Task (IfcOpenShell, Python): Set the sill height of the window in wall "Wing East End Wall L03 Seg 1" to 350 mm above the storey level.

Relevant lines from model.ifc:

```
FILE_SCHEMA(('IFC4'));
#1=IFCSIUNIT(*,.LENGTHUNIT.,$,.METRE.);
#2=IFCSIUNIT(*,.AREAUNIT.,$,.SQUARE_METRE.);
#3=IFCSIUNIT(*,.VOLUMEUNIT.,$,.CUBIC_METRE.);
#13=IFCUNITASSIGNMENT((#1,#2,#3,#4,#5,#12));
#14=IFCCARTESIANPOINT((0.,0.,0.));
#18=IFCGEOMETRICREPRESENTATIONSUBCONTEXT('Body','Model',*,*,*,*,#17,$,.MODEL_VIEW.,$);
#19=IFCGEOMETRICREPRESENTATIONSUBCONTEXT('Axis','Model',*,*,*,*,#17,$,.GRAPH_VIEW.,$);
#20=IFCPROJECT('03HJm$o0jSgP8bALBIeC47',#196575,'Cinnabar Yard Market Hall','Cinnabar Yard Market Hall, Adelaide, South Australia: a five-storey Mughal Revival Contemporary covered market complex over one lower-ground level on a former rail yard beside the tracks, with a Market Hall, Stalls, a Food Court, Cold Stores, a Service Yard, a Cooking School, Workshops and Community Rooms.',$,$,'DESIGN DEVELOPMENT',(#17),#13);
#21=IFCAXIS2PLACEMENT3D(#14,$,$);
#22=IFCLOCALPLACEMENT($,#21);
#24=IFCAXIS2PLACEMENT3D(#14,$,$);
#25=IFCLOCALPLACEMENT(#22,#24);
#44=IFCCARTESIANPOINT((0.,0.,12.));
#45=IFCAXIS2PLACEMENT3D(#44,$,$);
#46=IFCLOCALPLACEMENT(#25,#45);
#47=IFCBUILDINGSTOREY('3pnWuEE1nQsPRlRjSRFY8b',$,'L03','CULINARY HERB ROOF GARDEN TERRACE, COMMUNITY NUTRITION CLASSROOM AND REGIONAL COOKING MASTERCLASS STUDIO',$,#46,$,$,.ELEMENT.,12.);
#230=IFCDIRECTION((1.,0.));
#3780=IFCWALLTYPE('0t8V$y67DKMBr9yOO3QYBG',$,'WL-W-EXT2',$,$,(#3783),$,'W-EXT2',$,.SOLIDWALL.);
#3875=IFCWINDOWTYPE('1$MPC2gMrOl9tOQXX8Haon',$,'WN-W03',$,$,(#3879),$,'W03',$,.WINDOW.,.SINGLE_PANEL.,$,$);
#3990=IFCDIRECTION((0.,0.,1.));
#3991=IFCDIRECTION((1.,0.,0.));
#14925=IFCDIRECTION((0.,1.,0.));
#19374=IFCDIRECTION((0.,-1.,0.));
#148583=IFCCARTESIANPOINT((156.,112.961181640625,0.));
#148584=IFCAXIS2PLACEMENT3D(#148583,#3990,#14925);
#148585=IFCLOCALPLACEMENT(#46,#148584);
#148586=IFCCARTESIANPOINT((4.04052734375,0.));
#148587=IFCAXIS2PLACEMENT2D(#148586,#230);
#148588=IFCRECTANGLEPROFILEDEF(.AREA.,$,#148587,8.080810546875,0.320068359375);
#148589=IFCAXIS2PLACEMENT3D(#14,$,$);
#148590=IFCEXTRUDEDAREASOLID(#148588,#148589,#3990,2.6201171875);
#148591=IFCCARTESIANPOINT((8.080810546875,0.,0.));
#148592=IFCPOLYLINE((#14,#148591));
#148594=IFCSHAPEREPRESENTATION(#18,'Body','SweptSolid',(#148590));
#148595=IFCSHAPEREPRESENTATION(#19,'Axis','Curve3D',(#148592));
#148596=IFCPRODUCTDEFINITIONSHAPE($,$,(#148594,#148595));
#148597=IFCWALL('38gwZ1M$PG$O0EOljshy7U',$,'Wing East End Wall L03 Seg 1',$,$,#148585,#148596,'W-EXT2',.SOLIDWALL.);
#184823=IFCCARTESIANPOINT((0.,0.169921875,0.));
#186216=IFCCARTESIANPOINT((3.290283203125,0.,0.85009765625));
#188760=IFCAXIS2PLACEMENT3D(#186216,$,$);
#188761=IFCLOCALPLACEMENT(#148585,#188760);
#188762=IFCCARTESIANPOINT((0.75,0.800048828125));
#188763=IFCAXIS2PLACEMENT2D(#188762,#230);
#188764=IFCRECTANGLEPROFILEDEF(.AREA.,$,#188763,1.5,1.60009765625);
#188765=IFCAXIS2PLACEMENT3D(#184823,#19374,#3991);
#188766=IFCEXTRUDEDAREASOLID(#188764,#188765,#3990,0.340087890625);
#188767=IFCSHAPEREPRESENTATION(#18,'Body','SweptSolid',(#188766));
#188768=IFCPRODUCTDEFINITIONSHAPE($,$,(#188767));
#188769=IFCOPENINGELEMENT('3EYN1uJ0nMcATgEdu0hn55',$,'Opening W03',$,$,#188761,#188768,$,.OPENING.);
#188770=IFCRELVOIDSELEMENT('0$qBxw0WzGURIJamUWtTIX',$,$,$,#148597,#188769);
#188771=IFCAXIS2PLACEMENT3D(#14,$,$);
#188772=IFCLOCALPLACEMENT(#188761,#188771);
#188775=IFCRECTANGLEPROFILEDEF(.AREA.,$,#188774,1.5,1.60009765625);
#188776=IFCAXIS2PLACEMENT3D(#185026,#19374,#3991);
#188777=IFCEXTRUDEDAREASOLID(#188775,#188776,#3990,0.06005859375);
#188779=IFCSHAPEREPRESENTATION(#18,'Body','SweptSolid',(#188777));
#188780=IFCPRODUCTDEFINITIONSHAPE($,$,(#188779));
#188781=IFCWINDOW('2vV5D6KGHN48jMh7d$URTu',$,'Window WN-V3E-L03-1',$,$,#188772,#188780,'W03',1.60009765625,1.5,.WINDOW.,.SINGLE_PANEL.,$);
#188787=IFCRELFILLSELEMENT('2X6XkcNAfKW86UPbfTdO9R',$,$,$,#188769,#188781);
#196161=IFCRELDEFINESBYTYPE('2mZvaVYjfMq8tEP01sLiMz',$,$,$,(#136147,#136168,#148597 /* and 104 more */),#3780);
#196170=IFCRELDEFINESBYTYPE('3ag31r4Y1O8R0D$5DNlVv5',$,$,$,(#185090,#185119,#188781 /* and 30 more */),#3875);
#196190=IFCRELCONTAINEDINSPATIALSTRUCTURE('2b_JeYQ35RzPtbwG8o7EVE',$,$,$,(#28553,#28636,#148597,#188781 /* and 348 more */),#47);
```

```python
import numpy as np
import ifcopenshell
import ifcopenshell.api.geometry
import ifcopenshell.geom
import ifcopenshell.util.element
import ifcopenshell.util.placement
import ifcopenshell.util.shape
import ifcopenshell.util.unit

model = ifcopenshell.open("model.ifc")
unit_scale = ifcopenshell.util.unit.calculate_unit_scale(model)

window = model.by_guid("2vV5D6KGHN48jMh7d$URTu")
opening = window.FillsVoids[0].RelatingOpeningElement
storey = ifcopenshell.util.element.get_container(window, ifc_class="IfcBuildingStorey")
level = ifcopenshell.util.placement.get_local_placement(storey.ObjectPlacement)[2, 3]

# The opening's origin need not be at the sill, so measure its lowest point.
shape = ifcopenshell.geom.create_shape(ifcopenshell.geom.settings(), opening)
bottom = ifcopenshell.util.shape.get_shape_bottom_elevation(shape, shape.geometry) / unit_scale
dz = level + 0.35 - bottom

shift = np.array([0.0, 0.0, dz])
# The window is placed relative to its opening, so it follows when the opening moves.
matrix = ifcopenshell.util.placement.get_local_placement(opening.ObjectPlacement)
matrix[:3, 3] += shift
ifcopenshell.api.geometry.edit_object_placement(
    model, product=opening, matrix=matrix, is_si=False, should_transform_children=True
)

print(f"moved by {dz * unit_scale:+.3f} m")

model.write("model_edited.ifc")
```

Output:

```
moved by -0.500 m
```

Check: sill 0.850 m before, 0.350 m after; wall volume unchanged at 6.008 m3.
